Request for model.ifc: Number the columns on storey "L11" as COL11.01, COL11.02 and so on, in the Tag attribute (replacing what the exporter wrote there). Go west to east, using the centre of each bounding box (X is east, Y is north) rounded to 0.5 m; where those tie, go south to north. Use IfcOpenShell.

First a look at what the model holds.

```python
import ifcopenshell
import ifcopenshell.util.element
import ifcopenshell.util.placement

model = ifcopenshell.open("model.ifc")
print(model.schema)
storey = next(s for s in model.by_type("IfcBuildingStorey") if s.Name == "L11")
columns = [e for e in ifcopenshell.util.element.get_decomposition(storey) if e.is_a("IfcColumn")]
for e in sorted(columns, key=lambda e: e.id()):
    origin = ifcopenshell.util.placement.get_local_placement(e.ObjectPlacement)[:3, 3]
    print(e.id(), e.Tag, e.Name, origin.round(2) + 0.0, sep=" | ")
```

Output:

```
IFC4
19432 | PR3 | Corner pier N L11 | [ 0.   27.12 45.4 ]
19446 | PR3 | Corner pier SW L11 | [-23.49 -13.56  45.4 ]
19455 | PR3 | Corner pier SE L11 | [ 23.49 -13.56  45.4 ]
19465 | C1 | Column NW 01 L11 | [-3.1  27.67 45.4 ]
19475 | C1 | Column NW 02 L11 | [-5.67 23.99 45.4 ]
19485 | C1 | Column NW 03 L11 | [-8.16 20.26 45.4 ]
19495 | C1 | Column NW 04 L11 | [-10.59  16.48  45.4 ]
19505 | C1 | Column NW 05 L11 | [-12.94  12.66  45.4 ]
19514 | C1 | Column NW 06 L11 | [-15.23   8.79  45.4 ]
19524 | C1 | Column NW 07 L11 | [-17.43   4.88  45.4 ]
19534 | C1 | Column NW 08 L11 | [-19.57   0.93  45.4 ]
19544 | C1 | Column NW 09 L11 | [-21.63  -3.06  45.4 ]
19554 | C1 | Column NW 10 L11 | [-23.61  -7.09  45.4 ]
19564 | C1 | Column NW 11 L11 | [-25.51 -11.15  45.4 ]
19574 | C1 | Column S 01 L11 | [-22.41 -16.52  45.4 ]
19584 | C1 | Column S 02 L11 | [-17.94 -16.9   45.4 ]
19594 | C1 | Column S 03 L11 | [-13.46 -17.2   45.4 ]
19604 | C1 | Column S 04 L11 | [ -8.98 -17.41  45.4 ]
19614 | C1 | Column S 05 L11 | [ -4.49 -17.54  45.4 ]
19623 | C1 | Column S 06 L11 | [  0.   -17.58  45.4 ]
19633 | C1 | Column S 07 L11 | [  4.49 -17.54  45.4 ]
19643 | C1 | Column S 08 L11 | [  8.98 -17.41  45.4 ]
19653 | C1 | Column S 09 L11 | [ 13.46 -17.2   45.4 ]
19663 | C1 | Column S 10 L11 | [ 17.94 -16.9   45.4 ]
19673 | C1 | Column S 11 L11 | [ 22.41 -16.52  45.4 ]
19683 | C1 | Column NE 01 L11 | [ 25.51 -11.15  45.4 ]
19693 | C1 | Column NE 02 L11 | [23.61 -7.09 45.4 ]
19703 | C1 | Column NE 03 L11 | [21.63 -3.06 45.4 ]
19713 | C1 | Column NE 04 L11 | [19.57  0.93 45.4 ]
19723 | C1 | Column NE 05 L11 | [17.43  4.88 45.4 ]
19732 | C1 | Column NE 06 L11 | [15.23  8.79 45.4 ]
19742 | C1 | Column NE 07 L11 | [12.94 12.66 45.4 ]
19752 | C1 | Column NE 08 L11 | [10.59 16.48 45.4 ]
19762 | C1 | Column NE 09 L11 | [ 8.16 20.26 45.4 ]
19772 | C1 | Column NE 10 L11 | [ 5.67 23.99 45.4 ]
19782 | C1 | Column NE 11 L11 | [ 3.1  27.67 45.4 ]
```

```python
import ifcopenshell
import ifcopenshell.geom
import ifcopenshell.util.element
import ifcopenshell.util.shape

model = ifcopenshell.open("model.ifc")
settings = ifcopenshell.geom.settings()
settings.set("use-world-coords", True)


def centre(element):
    shape = ifcopenshell.geom.create_shape(settings, element)
    return ifcopenshell.util.shape.get_bbox_centroid(shape.geometry)


storey = next(s for s in model.by_type("IfcBuildingStorey") if s.Name == "L11")
columns = [e for e in ifcopenshell.util.element.get_decomposition(storey) if e.is_a("IfcColumn")]

# Insertion points can sit at a corner or the storey origin, so sort by the geometry (in metres).
centres = {e: centre(e) for e in columns}
columns.sort(key=lambda e: (round(centres[e][0] / 0.5), centres[e][1]))

for i, e in enumerate(columns, start=1):
    number = f"COL11.{i:02d}"
    e.Tag = number
    print(e.id(), number)

model.write("model_edited.ifc")
```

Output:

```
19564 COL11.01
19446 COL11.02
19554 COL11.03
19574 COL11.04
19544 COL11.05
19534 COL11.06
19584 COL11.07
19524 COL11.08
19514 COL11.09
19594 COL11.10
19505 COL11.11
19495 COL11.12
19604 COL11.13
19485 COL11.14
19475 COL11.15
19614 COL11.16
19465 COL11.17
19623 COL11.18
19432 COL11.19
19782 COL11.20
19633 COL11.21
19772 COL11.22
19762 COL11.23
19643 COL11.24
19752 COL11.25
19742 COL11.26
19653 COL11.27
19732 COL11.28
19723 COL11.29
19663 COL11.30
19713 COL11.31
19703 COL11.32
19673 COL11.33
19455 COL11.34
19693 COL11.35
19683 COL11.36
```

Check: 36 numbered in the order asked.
